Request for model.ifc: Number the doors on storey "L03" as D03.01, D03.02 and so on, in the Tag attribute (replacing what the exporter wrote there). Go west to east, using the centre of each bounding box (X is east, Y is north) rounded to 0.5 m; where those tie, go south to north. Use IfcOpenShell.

First a look at what the model holds.

```python
import ifcopenshell
import ifcopenshell.util.element
import ifcopenshell.util.placement

model = ifcopenshell.open("model.ifc")
print(model.schema)
storey = next(s for s in model.by_type("IfcBuildingStorey") if s.Name == "L03")
doors = [e for e in ifcopenshell.util.element.get_decomposition(storey) if e.is_a("IfcDoor")]
for e in sorted(doors, key=lambda e: e.id()):
    origin = ifcopenshell.util.placement.get_local_placement(e.ObjectPlacement)[:3, 3]
    print(e.id(), e.Tag, e.Name, origin.round(2) + 0.0, sep=" | ")
```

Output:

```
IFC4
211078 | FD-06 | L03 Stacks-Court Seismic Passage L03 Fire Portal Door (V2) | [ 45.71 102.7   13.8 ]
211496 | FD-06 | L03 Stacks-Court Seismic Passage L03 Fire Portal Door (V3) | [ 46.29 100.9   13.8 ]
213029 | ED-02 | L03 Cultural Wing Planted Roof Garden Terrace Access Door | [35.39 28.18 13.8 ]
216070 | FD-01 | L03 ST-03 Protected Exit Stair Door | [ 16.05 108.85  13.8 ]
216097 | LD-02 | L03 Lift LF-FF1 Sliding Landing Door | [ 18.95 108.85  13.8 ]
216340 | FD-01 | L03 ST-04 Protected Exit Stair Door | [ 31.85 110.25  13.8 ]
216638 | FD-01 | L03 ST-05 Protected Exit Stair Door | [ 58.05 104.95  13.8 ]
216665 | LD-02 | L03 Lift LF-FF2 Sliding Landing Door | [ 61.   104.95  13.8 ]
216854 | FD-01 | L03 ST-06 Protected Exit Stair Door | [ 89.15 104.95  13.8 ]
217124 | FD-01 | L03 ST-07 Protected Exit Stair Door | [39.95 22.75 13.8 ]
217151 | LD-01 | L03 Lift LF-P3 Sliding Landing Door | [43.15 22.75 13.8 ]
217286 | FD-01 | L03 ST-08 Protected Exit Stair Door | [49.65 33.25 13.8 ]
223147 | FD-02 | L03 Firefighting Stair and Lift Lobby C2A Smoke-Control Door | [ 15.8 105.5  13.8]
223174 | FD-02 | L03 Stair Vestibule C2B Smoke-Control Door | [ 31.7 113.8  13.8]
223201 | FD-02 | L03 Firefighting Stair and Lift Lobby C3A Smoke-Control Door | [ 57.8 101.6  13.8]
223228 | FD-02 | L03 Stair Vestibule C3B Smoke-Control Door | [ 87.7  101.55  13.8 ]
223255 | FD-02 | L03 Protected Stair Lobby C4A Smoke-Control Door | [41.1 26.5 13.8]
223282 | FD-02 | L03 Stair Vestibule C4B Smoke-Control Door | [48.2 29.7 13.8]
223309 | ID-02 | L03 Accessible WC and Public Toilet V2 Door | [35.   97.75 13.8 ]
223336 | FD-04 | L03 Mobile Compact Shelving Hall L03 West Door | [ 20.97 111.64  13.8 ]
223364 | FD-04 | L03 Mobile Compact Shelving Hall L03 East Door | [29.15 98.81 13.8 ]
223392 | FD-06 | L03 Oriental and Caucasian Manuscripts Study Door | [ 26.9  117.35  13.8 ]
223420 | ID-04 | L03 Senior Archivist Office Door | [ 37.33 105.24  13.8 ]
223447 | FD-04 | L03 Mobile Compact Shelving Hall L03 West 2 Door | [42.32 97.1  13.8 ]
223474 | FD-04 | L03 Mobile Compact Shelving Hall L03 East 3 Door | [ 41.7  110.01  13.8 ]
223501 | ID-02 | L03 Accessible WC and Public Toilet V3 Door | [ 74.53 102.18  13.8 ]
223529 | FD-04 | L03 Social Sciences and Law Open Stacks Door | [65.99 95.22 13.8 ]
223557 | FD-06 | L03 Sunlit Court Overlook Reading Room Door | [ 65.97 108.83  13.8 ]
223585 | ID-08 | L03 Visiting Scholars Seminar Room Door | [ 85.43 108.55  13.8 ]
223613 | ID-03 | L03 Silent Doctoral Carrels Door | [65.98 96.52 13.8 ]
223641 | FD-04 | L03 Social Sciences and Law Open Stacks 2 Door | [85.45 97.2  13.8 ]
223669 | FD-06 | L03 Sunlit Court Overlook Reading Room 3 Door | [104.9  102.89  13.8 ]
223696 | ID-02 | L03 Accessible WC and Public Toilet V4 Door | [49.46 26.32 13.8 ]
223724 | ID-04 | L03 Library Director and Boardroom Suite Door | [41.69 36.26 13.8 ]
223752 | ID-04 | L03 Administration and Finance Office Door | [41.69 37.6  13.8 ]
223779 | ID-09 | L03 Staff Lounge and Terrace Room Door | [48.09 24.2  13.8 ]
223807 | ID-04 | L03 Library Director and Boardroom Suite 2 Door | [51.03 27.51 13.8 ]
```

```python
import ifcopenshell
import ifcopenshell.geom
import ifcopenshell.util.element
import ifcopenshell.util.shape

model = ifcopenshell.open("model.ifc")
settings = ifcopenshell.geom.settings()
settings.set("use-world-coords", True)


def centre(element):
    shape = ifcopenshell.geom.create_shape(settings, element)
    return ifcopenshell.util.shape.get_bbox_centroid(shape.geometry)


storey = next(s for s in model.by_type("IfcBuildingStorey") if s.Name == "L03")
doors = [e for e in ifcopenshell.util.element.get_decomposition(storey) if e.is_a("IfcDoor")]

# Insertion points can sit at a corner or the storey origin, so sort by the geometry (in metres).
centres = {e: centre(e) for e in doors}
doors.sort(key=lambda e: (round(centres[e][0] / 0.5), centres[e][1]))

for i, e in enumerate(doors, start=1):
    number = f"D03.{i:02d}"
    e.Tag = number
    print(e.id(), number)

model.write("model_edited.ifc")
```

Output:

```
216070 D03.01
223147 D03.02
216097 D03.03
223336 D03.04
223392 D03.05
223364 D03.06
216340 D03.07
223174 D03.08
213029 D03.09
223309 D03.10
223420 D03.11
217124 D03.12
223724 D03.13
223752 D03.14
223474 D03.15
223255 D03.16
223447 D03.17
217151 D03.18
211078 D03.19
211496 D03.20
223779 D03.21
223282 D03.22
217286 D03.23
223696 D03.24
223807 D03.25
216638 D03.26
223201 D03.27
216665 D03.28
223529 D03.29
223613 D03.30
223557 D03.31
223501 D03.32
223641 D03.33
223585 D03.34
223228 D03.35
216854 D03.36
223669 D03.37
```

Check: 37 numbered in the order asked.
